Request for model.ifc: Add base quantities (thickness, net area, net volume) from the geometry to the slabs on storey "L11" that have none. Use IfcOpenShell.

First a look at what the model holds.

```python
import ifcopenshell
import ifcopenshell.util.element
import ifcopenshell.util.unit

model = ifcopenshell.open("model.ifc")
print(model.schema)
for unit_type in ("LENGTHUNIT", "AREAUNIT", "VOLUMEUNIT"):
    print(unit_type, ifcopenshell.util.unit.calculate_unit_scale(model, unit_type))
storey = next(s for s in model.by_type("IfcBuildingStorey") if s.Name == "L11")
slabs = [e for e in ifcopenshell.util.element.get_decomposition(storey) if e.is_a("IfcSlab")]
for e in sorted(slabs, key=lambda e: e.id()):
    print(e.id(), e.is_a(), e.Name, list(ifcopenshell.util.element.get_psets(e, qtos_only=True)), sep=" | ")
```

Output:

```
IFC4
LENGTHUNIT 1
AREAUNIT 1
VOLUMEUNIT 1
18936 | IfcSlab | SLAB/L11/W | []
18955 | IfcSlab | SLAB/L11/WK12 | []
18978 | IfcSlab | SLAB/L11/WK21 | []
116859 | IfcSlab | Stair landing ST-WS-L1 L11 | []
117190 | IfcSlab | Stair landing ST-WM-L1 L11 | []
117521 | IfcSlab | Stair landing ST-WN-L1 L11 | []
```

```python
import ifcopenshell
import ifcopenshell.api.pset
import ifcopenshell.geom
import ifcopenshell.util.element
import ifcopenshell.util.shape
import ifcopenshell.util.unit

model = ifcopenshell.open("model.ifc")
unit_scale = ifcopenshell.util.unit.calculate_unit_scale(model)
area_scale = ifcopenshell.util.unit.calculate_unit_scale(model, "AREAUNIT")
volume_scale = ifcopenshell.util.unit.calculate_unit_scale(model, "VOLUMEUNIT")
settings = ifcopenshell.geom.settings()

storey = next(s for s in model.by_type("IfcBuildingStorey") if s.Name == "L11")
slabs = [e for e in ifcopenshell.util.element.get_decomposition(storey) if e.is_a("IfcSlab")]

for e in sorted(slabs, key=lambda e: e.id()):
    if ifcopenshell.util.element.get_psets(e, qtos_only=True, should_inherit=False):
        continue
    # Geometry comes back in metres, in the element's own axes.
    shape = ifcopenshell.geom.create_shape(settings, e)
    values = {
        "Width": ifcopenshell.util.shape.get_z(shape.geometry) / unit_scale,
        "NetArea": ifcopenshell.util.shape.get_footprint_area(shape.geometry) / area_scale,
        "NetVolume": ifcopenshell.util.shape.get_volume(shape.geometry) / volume_scale,
    }
    qto = ifcopenshell.api.pset.add_qto(model, product=e, name="Qto_SlabBaseQuantities")
    ifcopenshell.api.pset.edit_qto(model, qto=qto, properties=values)
    print(e.id(), {k: round(v, 3) for k, v in values.items()})

model.write("model-out.ifc")
```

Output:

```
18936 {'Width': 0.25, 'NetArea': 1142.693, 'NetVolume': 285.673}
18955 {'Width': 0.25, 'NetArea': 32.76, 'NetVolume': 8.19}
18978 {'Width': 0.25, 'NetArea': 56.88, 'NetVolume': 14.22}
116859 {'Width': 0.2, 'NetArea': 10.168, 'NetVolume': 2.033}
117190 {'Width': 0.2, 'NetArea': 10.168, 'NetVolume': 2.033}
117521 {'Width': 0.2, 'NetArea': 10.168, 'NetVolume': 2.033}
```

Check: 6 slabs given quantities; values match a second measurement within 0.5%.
